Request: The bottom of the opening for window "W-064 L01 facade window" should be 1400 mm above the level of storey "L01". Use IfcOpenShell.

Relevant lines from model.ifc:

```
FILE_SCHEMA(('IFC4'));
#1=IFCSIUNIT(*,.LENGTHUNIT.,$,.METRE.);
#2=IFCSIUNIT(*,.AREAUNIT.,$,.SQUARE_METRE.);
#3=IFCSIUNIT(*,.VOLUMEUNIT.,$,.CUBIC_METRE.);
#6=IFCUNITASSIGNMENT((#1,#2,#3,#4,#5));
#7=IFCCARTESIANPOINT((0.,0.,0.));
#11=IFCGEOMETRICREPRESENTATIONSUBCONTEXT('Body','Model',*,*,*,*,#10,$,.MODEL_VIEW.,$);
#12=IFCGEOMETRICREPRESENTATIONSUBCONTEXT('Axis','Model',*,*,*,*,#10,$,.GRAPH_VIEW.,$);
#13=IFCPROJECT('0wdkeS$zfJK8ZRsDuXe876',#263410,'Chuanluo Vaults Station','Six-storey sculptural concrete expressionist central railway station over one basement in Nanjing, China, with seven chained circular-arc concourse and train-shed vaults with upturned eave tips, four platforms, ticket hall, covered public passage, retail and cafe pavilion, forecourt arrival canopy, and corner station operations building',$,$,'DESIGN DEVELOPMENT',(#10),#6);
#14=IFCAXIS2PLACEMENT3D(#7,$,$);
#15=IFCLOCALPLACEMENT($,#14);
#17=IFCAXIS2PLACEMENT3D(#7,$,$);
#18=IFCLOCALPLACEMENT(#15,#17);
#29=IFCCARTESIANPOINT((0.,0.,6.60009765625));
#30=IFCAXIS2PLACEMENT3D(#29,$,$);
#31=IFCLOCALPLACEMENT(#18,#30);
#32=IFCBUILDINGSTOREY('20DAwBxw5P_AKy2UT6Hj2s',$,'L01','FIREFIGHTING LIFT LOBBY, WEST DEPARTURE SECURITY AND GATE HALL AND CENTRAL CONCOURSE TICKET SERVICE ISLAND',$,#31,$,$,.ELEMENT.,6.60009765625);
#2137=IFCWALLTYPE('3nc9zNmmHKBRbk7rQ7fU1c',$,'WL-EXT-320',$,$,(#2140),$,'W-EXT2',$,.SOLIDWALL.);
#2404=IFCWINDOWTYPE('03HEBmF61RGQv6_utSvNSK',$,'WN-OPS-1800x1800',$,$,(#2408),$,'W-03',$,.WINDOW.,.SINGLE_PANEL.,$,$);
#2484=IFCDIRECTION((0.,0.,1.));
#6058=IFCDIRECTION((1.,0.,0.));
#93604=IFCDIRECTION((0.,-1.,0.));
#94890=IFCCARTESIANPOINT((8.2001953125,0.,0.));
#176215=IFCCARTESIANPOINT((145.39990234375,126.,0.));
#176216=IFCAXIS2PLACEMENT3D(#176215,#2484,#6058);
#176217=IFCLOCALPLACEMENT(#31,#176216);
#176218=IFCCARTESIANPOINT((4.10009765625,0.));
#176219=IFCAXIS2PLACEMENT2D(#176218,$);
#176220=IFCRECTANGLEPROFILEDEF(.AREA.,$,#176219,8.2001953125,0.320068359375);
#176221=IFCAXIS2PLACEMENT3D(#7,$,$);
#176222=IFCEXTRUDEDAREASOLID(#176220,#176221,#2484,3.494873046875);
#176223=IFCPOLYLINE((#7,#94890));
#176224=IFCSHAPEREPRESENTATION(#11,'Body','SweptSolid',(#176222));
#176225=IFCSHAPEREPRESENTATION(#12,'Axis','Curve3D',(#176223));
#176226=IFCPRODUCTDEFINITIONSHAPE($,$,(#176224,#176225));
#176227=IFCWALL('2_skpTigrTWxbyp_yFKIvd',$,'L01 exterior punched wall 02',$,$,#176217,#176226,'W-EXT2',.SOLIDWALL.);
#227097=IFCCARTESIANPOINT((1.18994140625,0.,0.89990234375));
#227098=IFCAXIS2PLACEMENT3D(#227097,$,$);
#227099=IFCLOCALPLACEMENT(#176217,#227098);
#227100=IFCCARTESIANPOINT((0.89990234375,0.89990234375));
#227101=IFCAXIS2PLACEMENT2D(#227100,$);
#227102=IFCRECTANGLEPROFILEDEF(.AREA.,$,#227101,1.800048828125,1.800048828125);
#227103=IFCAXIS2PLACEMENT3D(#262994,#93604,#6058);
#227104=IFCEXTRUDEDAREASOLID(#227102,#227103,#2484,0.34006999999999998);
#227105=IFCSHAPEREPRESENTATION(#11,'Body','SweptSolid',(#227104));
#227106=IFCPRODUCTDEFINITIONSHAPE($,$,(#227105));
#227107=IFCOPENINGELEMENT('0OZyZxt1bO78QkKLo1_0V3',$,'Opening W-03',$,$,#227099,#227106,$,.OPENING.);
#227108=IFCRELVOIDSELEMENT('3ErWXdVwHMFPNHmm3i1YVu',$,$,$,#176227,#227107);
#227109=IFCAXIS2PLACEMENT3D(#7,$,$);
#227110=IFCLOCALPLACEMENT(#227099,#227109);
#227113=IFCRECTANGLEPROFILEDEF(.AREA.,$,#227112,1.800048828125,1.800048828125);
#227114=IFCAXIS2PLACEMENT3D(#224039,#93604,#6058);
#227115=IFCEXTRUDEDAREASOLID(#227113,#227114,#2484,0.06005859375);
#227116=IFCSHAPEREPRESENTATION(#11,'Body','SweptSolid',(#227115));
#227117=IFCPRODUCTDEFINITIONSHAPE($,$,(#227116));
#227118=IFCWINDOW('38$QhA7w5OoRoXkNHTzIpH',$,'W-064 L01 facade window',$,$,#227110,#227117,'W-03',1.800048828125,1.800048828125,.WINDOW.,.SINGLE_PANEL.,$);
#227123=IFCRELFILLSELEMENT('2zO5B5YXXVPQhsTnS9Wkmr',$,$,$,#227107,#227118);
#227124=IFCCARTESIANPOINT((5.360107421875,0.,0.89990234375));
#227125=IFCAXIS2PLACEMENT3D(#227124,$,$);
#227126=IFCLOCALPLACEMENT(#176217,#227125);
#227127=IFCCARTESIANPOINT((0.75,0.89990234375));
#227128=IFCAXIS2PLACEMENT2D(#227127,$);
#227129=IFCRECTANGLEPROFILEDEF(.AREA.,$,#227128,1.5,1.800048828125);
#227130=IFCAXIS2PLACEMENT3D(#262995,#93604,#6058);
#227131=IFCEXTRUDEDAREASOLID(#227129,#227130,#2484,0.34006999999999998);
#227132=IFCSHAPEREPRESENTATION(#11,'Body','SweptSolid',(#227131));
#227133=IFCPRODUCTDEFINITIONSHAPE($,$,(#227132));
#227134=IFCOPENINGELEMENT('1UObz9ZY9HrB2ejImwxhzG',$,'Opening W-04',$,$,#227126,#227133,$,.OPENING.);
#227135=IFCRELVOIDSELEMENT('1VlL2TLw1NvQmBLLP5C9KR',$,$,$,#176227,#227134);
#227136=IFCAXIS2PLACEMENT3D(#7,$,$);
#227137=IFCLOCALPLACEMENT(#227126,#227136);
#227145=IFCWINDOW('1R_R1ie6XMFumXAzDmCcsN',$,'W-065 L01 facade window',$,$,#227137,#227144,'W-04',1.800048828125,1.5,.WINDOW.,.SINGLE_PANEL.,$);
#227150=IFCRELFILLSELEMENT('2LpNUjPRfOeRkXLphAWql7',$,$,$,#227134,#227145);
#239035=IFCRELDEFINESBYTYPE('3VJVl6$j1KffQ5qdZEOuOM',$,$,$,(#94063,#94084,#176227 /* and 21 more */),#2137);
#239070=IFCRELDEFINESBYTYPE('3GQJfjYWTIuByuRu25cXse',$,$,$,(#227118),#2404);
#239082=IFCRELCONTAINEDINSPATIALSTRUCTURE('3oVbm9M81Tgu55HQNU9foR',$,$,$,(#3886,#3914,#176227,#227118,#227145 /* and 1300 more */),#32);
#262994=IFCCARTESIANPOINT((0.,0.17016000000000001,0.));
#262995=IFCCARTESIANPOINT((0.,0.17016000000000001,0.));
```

```python
import numpy as np
import ifcopenshell
import ifcopenshell.api.geometry
import ifcopenshell.geom
import ifcopenshell.util.element
import ifcopenshell.util.placement
import ifcopenshell.util.shape
import ifcopenshell.util.unit

model = ifcopenshell.open("model.ifc")
unit_scale = ifcopenshell.util.unit.calculate_unit_scale(model)

window = model.by_id(227118)
opening = window.FillsVoids[0].RelatingOpeningElement
storey = ifcopenshell.util.element.get_container(window, ifc_class="IfcBuildingStorey")
level = ifcopenshell.util.placement.get_local_placement(storey.ObjectPlacement)[2, 3]

# The opening's origin need not be at the sill, so measure its lowest point.
shape = ifcopenshell.geom.create_shape(ifcopenshell.geom.settings(), opening)
bottom = ifcopenshell.util.shape.get_shape_bottom_elevation(shape, shape.geometry) / unit_scale
dz = level + 1.4 / unit_scale - bottom

shift = np.array([0.0, 0.0, dz])
# The window is placed relative to its opening, so it follows when the opening moves.
matrix = ifcopenshell.util.placement.get_local_placement(opening.ObjectPlacement)
matrix[:3, 3] += shift
ifcopenshell.api.geometry.edit_object_placement(
    model, product=opening, matrix=matrix, is_si=False, should_transform_children=True
)

print(f"moved by {dz * unit_scale:+.3f} m")

model.write("model_v2.ifc")
```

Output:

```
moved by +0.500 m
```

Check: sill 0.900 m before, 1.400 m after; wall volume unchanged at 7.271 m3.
